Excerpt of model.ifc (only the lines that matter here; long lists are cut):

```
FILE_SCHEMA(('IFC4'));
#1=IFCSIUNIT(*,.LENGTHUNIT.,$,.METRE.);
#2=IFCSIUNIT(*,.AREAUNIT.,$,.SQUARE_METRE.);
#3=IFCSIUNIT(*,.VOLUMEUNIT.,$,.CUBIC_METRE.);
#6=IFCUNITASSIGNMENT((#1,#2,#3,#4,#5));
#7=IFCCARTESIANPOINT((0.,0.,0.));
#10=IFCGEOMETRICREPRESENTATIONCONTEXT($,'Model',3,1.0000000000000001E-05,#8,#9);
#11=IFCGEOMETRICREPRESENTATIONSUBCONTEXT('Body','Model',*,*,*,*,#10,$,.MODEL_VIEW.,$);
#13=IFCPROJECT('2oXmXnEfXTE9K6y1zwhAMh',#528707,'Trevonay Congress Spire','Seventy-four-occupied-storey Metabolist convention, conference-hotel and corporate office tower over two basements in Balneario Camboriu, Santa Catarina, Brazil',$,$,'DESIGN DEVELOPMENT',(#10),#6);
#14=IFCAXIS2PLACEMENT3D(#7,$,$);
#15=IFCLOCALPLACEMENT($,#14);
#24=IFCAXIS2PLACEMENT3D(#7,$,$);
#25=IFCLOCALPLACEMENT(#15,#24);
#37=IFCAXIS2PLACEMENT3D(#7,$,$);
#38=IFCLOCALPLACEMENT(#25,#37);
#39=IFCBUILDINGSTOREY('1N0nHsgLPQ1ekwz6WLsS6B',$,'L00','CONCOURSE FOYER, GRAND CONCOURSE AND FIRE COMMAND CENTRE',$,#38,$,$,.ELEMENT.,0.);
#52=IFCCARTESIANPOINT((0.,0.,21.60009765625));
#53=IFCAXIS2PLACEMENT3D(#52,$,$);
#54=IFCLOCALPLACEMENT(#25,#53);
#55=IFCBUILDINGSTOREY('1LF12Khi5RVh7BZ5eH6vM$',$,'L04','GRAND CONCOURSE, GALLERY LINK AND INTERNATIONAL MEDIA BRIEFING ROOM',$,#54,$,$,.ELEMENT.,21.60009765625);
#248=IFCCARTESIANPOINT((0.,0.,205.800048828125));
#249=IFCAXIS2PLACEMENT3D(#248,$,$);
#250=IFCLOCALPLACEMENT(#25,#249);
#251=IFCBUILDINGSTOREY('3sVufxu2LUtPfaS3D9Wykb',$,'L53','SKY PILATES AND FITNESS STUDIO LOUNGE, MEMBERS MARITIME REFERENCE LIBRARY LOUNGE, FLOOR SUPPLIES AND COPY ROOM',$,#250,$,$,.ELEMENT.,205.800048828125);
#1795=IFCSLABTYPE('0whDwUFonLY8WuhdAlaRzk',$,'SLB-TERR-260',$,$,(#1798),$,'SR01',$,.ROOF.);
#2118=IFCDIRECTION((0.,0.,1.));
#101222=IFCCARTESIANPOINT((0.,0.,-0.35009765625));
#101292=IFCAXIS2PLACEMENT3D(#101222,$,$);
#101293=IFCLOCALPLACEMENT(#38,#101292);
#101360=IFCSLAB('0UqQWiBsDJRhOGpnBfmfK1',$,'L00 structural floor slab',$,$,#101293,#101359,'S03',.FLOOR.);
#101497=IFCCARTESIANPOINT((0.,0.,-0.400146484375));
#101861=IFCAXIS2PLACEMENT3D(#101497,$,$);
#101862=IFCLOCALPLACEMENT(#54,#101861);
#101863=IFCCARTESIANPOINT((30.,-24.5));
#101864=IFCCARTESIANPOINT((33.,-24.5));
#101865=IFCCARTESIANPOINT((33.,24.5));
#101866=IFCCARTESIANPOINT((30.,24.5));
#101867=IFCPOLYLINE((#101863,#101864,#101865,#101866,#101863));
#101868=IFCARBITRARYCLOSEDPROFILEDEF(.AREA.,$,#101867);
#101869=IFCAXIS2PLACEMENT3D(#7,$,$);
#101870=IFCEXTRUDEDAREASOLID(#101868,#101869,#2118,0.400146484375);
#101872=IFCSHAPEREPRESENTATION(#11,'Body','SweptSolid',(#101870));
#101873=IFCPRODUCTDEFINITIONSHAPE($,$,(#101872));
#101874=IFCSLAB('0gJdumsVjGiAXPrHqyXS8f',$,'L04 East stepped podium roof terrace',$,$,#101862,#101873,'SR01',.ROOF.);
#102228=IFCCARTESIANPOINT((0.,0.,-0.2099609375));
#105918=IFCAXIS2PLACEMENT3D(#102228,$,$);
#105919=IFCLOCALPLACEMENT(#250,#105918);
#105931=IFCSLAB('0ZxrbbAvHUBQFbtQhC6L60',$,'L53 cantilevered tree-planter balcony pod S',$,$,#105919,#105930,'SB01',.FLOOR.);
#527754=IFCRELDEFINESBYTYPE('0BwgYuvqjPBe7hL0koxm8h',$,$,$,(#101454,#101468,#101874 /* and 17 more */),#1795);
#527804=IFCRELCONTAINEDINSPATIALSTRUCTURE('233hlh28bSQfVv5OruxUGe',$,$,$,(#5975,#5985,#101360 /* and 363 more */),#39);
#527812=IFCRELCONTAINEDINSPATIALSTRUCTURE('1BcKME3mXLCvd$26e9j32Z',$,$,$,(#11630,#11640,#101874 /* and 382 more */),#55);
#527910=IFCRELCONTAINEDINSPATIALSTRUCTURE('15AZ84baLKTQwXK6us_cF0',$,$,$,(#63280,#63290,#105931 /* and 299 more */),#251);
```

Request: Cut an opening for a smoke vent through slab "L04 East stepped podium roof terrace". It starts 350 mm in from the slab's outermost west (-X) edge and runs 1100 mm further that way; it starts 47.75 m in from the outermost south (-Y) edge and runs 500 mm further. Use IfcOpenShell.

```python
import numpy as np
import ifcopenshell
import ifcopenshell.api.feature
import ifcopenshell.api.geometry
import ifcopenshell.api.root
import ifcopenshell.geom
import ifcopenshell.util.placement
import ifcopenshell.util.representation
import ifcopenshell.util.shape
import ifcopenshell.util.unit

model = ifcopenshell.open("model.ifc")
unit_scale = ifcopenshell.util.unit.calculate_unit_scale(model)
settings = ifcopenshell.geom.settings()


def volume(element):
    """Net volume in cubic metres, openings subtracted."""
    shape = ifcopenshell.geom.create_shape(settings, element)
    return ifcopenshell.util.shape.get_volume(shape.geometry)


slab = model.by_guid("0gJdumsVjGiAXPrHqyXS8f")
before = volume(slab)

# Extent in the slab's own axes, in metres. The edges named are its -X and -Y sides.
slab_shape = ifcopenshell.geom.create_shape(settings, slab)
vertices = ifcopenshell.util.shape.get_vertices(slab_shape.geometry)
x_min, y_min, bottom = vertices.min(axis=0)
top = vertices[:, 2].max()

opening = ifcopenshell.api.root.create_entity(model, ifc_class="IfcOpeningElement", name="Smoke vent opening", predefined_type="OPENING")
context = ifcopenshell.util.representation.get_context(model, "Model", "Body", "MODEL_VIEW")
width, depth = 1.1, 0.5
outline = [(0.0, 0.0), (width, 0.0), (width, depth), (0.0, depth), (0.0, 0.0)]
# Overshoot both faces by 50 mm so the cut is clean.
shape = ifcopenshell.api.geometry.add_slab_representation(
    model, context=context, depth=top - bottom + 0.1, polyline=outline
)
ifcopenshell.api.geometry.assign_representation(model, product=opening, representation=shape)

matrix = ifcopenshell.util.placement.get_local_placement(slab.ObjectPlacement)
matrix[:, 3] = matrix @ np.append(np.array([x_min + 0.35, y_min + 47.75, bottom - 0.05]) / unit_scale, 1.0)
ifcopenshell.api.geometry.edit_object_placement(model, product=opening, matrix=matrix, is_si=False)
ifcopenshell.api.feature.add_feature(model, feature=opening, element=slab)

after = volume(slab)

print(f"slab volume {before:.3f} -> {after:.3f} m3")

model.write("model-out.ifc")
```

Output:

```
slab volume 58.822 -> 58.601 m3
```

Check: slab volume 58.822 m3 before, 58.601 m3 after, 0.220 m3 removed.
